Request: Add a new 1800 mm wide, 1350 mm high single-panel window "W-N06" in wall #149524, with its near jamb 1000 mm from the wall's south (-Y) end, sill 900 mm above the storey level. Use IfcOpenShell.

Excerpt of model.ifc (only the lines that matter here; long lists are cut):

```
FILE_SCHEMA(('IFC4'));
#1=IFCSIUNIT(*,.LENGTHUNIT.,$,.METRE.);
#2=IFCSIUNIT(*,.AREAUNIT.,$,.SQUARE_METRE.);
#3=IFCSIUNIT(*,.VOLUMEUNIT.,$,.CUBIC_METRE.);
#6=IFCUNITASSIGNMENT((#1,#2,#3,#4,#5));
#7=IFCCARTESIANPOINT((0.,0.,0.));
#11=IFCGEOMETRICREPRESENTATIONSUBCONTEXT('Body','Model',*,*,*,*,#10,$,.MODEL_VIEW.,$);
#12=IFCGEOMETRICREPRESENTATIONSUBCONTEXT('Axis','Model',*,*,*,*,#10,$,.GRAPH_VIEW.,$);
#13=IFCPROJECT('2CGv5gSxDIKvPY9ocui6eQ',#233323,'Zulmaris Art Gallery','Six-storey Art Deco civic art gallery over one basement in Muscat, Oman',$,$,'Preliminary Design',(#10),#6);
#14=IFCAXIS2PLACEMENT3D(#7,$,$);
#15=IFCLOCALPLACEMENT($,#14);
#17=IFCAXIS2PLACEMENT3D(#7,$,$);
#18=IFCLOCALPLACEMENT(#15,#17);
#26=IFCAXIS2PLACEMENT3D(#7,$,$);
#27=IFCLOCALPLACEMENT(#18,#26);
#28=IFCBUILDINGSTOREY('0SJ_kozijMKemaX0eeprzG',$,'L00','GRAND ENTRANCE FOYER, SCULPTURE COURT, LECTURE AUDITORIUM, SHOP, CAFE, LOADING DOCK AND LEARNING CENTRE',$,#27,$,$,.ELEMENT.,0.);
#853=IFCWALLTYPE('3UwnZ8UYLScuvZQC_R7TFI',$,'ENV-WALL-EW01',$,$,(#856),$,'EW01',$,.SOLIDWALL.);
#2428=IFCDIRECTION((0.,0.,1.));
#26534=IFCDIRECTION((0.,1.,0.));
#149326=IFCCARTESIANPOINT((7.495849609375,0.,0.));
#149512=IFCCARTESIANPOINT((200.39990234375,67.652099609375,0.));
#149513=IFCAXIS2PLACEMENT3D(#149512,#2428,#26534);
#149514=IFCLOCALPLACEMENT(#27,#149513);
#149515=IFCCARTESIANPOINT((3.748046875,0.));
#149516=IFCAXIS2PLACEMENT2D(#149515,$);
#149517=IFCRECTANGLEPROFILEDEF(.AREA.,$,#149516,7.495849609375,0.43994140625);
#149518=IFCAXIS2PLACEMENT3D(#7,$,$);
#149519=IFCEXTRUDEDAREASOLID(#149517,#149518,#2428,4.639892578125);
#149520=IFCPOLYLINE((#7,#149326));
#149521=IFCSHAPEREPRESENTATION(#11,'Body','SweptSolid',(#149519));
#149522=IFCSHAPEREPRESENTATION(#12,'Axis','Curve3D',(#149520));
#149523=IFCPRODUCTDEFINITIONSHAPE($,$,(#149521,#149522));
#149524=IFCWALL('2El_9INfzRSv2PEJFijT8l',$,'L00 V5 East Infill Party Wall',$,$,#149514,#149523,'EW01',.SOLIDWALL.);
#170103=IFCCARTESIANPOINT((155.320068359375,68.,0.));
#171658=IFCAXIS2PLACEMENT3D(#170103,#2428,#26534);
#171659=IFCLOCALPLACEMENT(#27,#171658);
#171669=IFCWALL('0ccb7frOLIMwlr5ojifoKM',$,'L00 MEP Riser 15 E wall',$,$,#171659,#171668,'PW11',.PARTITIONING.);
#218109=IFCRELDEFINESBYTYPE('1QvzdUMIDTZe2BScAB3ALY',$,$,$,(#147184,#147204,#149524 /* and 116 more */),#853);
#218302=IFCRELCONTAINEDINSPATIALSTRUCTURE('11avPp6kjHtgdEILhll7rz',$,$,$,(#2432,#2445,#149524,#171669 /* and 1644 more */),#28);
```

```python
import numpy as np
import ifcopenshell
import ifcopenshell.api.feature
import ifcopenshell.api.geometry
import ifcopenshell.api.root
import ifcopenshell.api.spatial
import ifcopenshell.geom
import ifcopenshell.util.element
import ifcopenshell.util.placement
import ifcopenshell.util.representation
import ifcopenshell.util.shape
import ifcopenshell.util.unit

model = ifcopenshell.open("model.ifc")
unit_scale = ifcopenshell.util.unit.calculate_unit_scale(model)
settings = ifcopenshell.geom.settings()


def volume(element):
    """Net volume in cubic metres, openings subtracted."""
    shape = ifcopenshell.geom.create_shape(settings, element)
    return ifcopenshell.util.shape.get_volume(shape.geometry)


wall = model.by_guid("2El_9INfzRSv2PEJFijT8l")
storey = ifcopenshell.util.element.get_container(wall, ifc_class="IfcBuildingStorey")
context = ifcopenshell.util.representation.get_context(model, "Model", "Body", "MODEL_VIEW")
before = volume(wall)

width, height, from_end, sill = 1.8, 1.35, 1, 0.9  # metres

# The wall runs along its own X axis, and the end named is its -X end.
wall_shape = ifcopenshell.geom.create_shape(settings, wall)
x, y, z = ifcopenshell.util.shape.get_vertices(wall_shape.geometry).T
start = x.min() + from_end
face, thickness = float(y.min()), float(y.max() - y.min())
wall_matrix = ifcopenshell.util.placement.get_local_placement(wall.ObjectPlacement)
level = ifcopenshell.util.placement.get_local_placement(storey.ObjectPlacement)[2, 3]


def in_wall(x, y):
    """Placement at x, y metres in the wall's axes, at sill height."""
    matrix = wall_matrix.copy()
    matrix[:, 3] = wall_matrix @ np.array([x / unit_scale, y / unit_scale, 0.0, 1.0])
    matrix[2, 3] = level + sill / unit_scale
    return matrix


# Opening: a box that overshoots both wall faces by 50 mm.
opening = ifcopenshell.api.root.create_entity(model, ifc_class="IfcOpeningElement", predefined_type="OPENING")
box = ifcopenshell.api.geometry.add_wall_representation(
    model, context=context, length=width, height=height, thickness=thickness + 0.1
)
ifcopenshell.api.geometry.assign_representation(model, product=opening, representation=box)
ifcopenshell.api.geometry.edit_object_placement(model, product=opening, matrix=in_wall(start, face - 0.05), is_si=False)
ifcopenshell.api.feature.add_feature(model, feature=opening, element=wall)

window = ifcopenshell.api.root.create_entity(model, ifc_class="IfcWindow", name="W-N06", predefined_type="WINDOW")
window.OverallWidth, window.OverallHeight = width / unit_scale, height / unit_scale
window.PartitioningType = "SINGLE_PANEL"
body = ifcopenshell.api.geometry.add_window_representation(
    model,
    context=context,
    overall_width=window.OverallWidth,
    overall_height=window.OverallHeight,
    partition_type="SINGLE_PANEL",
)
ifcopenshell.api.geometry.assign_representation(model, product=window, representation=body)
ifcopenshell.api.spatial.assign_container(model, products=[window], relating_structure=storey)
ifcopenshell.api.feature.add_filling(model, opening=opening, element=window)

# Centre the window in the wall's thickness.
ifcopenshell.api.geometry.edit_object_placement(model, product=window, matrix=in_wall(start, face), is_si=False)
window_shape = ifcopenshell.geom.create_shape(settings, window)
depth = ifcopenshell.util.shape.get_vertices(window_shape.geometry)[:, 1]
offset = face + thickness / 2 - (depth.min() + depth.max()) / 2
ifcopenshell.api.geometry.edit_object_placement(model, product=window, matrix=in_wall(start, offset), is_si=False)

after = volume(wall)

print(f"wall volume {before:.3f} -> {after:.3f} m3")

model.write("model_edited.ifc")
```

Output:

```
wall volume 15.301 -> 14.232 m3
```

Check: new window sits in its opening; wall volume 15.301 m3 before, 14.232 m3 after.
